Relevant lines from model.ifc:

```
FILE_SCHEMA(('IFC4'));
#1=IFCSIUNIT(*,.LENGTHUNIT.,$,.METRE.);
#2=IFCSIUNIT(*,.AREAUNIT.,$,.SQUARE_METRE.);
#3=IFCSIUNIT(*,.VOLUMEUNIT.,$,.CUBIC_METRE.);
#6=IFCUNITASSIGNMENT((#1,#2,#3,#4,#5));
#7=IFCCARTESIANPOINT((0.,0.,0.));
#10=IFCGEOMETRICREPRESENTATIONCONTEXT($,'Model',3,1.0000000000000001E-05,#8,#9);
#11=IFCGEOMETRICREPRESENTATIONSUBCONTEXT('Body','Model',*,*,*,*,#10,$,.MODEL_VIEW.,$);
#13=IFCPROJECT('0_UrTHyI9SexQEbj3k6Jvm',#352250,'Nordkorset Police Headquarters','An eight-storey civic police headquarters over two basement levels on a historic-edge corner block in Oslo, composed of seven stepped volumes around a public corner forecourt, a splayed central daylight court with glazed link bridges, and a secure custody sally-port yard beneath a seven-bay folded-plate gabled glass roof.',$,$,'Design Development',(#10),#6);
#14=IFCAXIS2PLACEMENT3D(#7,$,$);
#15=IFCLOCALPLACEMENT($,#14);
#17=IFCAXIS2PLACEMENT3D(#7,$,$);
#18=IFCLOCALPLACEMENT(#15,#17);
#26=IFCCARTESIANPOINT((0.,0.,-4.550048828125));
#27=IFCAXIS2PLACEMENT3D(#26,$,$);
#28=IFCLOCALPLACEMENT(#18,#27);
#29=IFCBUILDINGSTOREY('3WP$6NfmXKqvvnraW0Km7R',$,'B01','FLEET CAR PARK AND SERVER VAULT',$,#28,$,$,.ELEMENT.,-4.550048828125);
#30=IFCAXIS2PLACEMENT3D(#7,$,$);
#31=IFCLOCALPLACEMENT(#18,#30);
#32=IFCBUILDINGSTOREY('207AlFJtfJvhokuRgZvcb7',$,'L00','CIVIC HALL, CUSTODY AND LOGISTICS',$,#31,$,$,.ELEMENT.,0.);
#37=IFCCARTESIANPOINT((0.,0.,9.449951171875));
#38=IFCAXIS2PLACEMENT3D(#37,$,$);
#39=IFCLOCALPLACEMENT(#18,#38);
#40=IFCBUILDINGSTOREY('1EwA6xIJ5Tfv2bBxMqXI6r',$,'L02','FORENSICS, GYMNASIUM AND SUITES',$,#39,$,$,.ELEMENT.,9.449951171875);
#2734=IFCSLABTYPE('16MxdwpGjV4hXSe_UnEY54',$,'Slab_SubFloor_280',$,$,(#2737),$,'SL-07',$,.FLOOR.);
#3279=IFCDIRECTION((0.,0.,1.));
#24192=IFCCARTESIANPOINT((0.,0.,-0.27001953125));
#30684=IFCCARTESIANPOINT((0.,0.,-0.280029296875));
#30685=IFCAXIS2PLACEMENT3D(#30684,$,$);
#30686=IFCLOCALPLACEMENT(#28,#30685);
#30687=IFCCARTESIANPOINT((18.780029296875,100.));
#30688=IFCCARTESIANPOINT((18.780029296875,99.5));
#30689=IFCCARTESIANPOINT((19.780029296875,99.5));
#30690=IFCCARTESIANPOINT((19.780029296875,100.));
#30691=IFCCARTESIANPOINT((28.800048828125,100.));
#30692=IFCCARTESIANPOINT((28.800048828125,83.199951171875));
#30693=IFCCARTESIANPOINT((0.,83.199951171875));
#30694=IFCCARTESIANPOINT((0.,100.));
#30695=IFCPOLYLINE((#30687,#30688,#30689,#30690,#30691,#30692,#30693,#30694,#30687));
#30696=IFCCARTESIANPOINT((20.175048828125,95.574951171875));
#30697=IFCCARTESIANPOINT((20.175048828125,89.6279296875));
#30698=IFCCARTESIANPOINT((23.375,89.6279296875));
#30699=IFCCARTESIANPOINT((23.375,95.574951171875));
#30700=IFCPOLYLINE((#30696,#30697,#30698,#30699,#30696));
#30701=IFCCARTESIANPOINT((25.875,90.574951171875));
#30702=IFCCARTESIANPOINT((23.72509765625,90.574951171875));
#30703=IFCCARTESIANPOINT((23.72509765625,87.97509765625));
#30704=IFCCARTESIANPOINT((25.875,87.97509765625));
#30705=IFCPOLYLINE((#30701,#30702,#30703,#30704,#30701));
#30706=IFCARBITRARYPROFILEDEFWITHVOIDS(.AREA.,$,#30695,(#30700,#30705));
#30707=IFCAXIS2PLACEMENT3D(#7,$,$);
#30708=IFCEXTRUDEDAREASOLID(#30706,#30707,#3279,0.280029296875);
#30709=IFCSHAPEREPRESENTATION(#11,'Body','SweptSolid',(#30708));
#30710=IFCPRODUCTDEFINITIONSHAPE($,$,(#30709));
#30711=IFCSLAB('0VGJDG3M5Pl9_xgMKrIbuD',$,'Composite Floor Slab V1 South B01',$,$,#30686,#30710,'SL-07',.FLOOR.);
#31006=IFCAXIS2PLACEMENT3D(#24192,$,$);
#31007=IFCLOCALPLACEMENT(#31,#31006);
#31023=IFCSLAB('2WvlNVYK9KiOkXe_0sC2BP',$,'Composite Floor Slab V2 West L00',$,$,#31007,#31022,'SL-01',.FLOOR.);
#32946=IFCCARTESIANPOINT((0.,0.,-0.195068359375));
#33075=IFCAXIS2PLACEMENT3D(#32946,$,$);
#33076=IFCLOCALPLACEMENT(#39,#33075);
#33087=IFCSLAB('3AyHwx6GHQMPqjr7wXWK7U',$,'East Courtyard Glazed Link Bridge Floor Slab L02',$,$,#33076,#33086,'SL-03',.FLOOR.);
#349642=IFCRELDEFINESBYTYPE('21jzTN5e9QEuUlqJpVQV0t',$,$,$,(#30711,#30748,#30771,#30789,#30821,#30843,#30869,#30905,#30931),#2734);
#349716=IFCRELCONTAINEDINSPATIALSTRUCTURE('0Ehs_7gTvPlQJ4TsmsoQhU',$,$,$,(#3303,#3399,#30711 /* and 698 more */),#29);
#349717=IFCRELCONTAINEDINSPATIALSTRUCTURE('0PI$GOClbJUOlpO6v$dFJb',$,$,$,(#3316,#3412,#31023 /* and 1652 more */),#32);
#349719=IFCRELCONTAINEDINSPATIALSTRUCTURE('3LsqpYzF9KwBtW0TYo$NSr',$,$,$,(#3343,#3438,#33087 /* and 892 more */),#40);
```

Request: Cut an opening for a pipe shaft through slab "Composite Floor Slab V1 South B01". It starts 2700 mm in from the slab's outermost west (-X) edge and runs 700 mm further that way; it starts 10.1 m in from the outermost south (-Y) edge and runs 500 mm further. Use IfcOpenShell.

```python
import numpy as np
import ifcopenshell
import ifcopenshell.api.feature
import ifcopenshell.api.geometry
import ifcopenshell.api.root
import ifcopenshell.geom
import ifcopenshell.util.placement
import ifcopenshell.util.representation
import ifcopenshell.util.shape
import ifcopenshell.util.unit

model = ifcopenshell.open("model.ifc")
unit_scale = ifcopenshell.util.unit.calculate_unit_scale(model)
settings = ifcopenshell.geom.settings()


def volume(element):
    """Net volume in cubic metres, openings subtracted."""
    shape = ifcopenshell.geom.create_shape(settings, element)
    return ifcopenshell.util.shape.get_volume(shape.geometry)


slab = model.by_id(30711)
before = volume(slab)

# Extent in the slab's own axes, in metres. The edges named are its -X and -Y sides.
slab_shape = ifcopenshell.geom.create_shape(settings, slab)
vertices = ifcopenshell.util.shape.get_vertices(slab_shape.geometry)
x_min, y_min, bottom = vertices.min(axis=0)
top = vertices[:, 2].max()

opening = ifcopenshell.api.root.create_entity(model, ifc_class="IfcOpeningElement", name="Pipe shaft opening", predefined_type="OPENING")
context = ifcopenshell.util.representation.get_context(model, "Model", "Body", "MODEL_VIEW")
width, depth = 0.7, 0.5
outline = [(0.0, 0.0), (width, 0.0), (width, depth), (0.0, depth), (0.0, 0.0)]
# Overshoot both faces by 50 mm so the cut is clean.
shape = ifcopenshell.api.geometry.add_slab_representation(
    model, context=context, depth=top - bottom + 0.1, polyline=outline
)
ifcopenshell.api.geometry.assign_representation(model, product=opening, representation=shape)

matrix = ifcopenshell.util.placement.get_local_placement(slab.ObjectPlacement)
matrix[:, 3] = matrix @ np.append(np.array([x_min + 2.7, y_min + 10.1, bottom - 0.05]) / unit_scale, 1.0)
ifcopenshell.api.geometry.edit_object_placement(model, product=opening, matrix=matrix, is_si=False)
ifcopenshell.api.feature.add_feature(model, feature=opening, element=slab)

after = volume(slab)

print(f"slab volume {before:.3f} -> {after:.3f} m3")

model.write("model-out.ifc")
```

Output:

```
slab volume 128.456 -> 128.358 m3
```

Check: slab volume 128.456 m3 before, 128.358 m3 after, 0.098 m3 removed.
